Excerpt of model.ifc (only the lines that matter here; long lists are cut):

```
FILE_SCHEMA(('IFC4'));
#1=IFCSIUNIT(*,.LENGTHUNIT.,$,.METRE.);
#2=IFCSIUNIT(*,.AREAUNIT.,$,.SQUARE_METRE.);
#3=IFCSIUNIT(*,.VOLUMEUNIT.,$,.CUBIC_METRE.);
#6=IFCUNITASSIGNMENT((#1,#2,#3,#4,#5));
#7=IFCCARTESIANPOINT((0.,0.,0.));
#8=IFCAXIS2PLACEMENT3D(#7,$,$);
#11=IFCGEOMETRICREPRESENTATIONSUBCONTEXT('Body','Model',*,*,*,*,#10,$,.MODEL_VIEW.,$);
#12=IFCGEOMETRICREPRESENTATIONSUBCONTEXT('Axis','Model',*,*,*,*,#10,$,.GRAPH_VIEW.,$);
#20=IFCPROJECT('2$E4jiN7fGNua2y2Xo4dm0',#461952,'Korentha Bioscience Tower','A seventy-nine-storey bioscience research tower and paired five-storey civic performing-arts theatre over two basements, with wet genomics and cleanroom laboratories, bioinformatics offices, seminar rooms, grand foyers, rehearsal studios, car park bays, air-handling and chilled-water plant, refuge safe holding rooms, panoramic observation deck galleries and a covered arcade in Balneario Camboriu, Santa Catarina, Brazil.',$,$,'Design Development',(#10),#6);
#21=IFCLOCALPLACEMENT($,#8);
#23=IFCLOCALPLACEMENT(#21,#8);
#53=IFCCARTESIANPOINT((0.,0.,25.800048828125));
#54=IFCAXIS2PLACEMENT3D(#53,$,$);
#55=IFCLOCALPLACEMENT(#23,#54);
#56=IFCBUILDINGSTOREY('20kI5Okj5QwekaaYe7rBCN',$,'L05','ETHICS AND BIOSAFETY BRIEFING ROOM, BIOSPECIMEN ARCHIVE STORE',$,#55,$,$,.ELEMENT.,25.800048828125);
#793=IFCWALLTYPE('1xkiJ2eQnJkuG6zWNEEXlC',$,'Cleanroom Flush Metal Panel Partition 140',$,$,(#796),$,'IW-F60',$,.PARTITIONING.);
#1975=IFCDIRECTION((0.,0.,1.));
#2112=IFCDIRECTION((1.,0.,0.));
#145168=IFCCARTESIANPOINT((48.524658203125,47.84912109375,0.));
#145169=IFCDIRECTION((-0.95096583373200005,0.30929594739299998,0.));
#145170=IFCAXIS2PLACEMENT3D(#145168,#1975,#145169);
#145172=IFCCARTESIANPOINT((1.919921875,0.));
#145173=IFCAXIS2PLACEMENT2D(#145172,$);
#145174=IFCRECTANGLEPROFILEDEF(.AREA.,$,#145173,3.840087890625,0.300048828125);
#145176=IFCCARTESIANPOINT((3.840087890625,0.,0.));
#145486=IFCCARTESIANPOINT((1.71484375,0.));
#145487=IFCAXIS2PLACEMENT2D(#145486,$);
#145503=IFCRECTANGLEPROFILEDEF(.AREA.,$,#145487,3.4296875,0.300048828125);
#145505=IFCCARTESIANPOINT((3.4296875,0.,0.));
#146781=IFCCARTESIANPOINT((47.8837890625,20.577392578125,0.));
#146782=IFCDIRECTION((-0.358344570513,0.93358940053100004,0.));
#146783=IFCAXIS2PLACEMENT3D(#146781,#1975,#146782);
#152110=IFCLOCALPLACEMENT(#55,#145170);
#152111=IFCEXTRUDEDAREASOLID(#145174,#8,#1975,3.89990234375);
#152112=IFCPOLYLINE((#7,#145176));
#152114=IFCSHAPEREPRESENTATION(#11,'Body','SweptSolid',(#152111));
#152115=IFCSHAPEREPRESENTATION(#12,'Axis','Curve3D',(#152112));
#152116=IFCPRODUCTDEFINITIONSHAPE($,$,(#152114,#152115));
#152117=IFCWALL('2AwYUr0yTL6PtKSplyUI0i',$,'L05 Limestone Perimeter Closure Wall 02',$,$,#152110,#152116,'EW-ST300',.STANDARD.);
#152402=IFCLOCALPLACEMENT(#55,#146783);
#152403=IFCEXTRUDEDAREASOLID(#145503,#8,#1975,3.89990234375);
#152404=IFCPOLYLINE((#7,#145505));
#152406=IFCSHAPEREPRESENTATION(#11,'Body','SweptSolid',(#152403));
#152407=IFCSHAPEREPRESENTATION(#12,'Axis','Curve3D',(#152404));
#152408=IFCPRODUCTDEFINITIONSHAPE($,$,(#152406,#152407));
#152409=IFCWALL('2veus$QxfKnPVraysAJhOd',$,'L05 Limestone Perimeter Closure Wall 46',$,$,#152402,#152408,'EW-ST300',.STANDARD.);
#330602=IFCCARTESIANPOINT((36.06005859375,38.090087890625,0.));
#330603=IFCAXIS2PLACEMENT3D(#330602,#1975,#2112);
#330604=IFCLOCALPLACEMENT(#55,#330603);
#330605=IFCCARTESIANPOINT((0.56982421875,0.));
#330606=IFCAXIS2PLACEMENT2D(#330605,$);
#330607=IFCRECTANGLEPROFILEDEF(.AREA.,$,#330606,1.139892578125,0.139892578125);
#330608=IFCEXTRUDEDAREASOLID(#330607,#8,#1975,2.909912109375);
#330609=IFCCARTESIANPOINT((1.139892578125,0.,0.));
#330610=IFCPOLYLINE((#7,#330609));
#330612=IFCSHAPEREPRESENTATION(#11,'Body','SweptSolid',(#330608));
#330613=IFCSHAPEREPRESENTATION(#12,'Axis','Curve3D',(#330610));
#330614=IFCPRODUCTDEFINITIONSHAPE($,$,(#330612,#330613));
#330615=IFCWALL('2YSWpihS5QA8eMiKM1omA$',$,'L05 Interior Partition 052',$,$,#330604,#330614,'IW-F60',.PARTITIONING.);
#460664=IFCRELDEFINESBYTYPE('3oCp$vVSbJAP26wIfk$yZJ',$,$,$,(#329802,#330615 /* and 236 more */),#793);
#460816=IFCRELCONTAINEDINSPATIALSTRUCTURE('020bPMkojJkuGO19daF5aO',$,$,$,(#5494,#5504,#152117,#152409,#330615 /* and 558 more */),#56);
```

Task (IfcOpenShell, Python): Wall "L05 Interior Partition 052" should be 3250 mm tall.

```python
import ifcopenshell
import ifcopenshell.geom
import ifcopenshell.util.representation
import ifcopenshell.util.shape

model = ifcopenshell.open("model.ifc")
settings = ifcopenshell.geom.settings()


def volume(element):
    """Net volume in cubic metres, openings subtracted."""
    shape = ifcopenshell.geom.create_shape(settings, element)
    return ifcopenshell.util.shape.get_volume(shape.geometry)


wall = model.by_id(330615)
before = volume(wall)

body = ifcopenshell.util.representation.get_representation(wall, "Model", "Body")
solid = body.Items[0]
old_height = solid.Depth
solid.Depth = 3.25
after = volume(wall)

print(f"height {old_height:g} -> {solid.Depth:g}, volume {before:.3f} -> {after:.3f} m3")

model.write("model-out.ifc")
```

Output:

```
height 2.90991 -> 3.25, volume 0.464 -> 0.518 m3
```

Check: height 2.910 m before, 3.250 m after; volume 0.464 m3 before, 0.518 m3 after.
